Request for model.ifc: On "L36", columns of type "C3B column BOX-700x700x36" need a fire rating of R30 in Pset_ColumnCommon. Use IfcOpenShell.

First a look at what the model holds.

```python
import ifcopenshell
import ifcopenshell.util.element

model = ifcopenshell.open("model.ifc")
print(model.schema)
storey = next(s for s in model.by_type("IfcBuildingStorey") if s.Name == "L36")
columns = [e for e in ifcopenshell.util.element.get_decomposition(storey) if e.is_a("IfcColumn")]
seen = {}
for e in columns:
    element_type = ifcopenshell.util.element.get_type(e)
    key = (element_type.Name if element_type != e and element_type else None, ifcopenshell.util.element.get_pset(e, "Pset_ColumnCommon", "FireRating"))
    seen[key] = seen.get(key, 0) + 1
for (name, value), count in sorted(seen.items(), key=str):
    print(count, "x", name, "|", value)
```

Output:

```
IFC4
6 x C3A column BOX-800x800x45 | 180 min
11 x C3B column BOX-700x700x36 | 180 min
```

```python
import ifcopenshell
import ifcopenshell.api.pset
import ifcopenshell.util.element

model = ifcopenshell.open("model.ifc")

storey = next(s for s in model.by_type("IfcBuildingStorey") if s.Name == "L36")
columns = [e for e in ifcopenshell.util.element.get_decomposition(storey) if e.is_a("IfcColumn")]

count = 0
for e in columns:
    element_type = ifcopenshell.util.element.get_type(e)
    if element_type in (None, e) or element_type.Name != "C3B column BOX-700x700x36":
        continue
    found = ifcopenshell.util.element.get_pset(e, "Pset_ColumnCommon", should_inherit=False)
    if found:
        pset = model.by_id(found["id"])
        if len(ifcopenshell.util.element.get_elements_by_pset(pset)) > 1:
            pset = ifcopenshell.api.pset.unshare_pset(model, products=[e], pset=pset)[0]
    else:
        pset = ifcopenshell.api.pset.add_pset(model, product=e, name="Pset_ColumnCommon")
    ifcopenshell.api.pset.edit_pset(model, pset=pset, properties={"FireRating": "R30"})
    count += 1

print(count, "columns updated")

model.write("model-out.ifc")
```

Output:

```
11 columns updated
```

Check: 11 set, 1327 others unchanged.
